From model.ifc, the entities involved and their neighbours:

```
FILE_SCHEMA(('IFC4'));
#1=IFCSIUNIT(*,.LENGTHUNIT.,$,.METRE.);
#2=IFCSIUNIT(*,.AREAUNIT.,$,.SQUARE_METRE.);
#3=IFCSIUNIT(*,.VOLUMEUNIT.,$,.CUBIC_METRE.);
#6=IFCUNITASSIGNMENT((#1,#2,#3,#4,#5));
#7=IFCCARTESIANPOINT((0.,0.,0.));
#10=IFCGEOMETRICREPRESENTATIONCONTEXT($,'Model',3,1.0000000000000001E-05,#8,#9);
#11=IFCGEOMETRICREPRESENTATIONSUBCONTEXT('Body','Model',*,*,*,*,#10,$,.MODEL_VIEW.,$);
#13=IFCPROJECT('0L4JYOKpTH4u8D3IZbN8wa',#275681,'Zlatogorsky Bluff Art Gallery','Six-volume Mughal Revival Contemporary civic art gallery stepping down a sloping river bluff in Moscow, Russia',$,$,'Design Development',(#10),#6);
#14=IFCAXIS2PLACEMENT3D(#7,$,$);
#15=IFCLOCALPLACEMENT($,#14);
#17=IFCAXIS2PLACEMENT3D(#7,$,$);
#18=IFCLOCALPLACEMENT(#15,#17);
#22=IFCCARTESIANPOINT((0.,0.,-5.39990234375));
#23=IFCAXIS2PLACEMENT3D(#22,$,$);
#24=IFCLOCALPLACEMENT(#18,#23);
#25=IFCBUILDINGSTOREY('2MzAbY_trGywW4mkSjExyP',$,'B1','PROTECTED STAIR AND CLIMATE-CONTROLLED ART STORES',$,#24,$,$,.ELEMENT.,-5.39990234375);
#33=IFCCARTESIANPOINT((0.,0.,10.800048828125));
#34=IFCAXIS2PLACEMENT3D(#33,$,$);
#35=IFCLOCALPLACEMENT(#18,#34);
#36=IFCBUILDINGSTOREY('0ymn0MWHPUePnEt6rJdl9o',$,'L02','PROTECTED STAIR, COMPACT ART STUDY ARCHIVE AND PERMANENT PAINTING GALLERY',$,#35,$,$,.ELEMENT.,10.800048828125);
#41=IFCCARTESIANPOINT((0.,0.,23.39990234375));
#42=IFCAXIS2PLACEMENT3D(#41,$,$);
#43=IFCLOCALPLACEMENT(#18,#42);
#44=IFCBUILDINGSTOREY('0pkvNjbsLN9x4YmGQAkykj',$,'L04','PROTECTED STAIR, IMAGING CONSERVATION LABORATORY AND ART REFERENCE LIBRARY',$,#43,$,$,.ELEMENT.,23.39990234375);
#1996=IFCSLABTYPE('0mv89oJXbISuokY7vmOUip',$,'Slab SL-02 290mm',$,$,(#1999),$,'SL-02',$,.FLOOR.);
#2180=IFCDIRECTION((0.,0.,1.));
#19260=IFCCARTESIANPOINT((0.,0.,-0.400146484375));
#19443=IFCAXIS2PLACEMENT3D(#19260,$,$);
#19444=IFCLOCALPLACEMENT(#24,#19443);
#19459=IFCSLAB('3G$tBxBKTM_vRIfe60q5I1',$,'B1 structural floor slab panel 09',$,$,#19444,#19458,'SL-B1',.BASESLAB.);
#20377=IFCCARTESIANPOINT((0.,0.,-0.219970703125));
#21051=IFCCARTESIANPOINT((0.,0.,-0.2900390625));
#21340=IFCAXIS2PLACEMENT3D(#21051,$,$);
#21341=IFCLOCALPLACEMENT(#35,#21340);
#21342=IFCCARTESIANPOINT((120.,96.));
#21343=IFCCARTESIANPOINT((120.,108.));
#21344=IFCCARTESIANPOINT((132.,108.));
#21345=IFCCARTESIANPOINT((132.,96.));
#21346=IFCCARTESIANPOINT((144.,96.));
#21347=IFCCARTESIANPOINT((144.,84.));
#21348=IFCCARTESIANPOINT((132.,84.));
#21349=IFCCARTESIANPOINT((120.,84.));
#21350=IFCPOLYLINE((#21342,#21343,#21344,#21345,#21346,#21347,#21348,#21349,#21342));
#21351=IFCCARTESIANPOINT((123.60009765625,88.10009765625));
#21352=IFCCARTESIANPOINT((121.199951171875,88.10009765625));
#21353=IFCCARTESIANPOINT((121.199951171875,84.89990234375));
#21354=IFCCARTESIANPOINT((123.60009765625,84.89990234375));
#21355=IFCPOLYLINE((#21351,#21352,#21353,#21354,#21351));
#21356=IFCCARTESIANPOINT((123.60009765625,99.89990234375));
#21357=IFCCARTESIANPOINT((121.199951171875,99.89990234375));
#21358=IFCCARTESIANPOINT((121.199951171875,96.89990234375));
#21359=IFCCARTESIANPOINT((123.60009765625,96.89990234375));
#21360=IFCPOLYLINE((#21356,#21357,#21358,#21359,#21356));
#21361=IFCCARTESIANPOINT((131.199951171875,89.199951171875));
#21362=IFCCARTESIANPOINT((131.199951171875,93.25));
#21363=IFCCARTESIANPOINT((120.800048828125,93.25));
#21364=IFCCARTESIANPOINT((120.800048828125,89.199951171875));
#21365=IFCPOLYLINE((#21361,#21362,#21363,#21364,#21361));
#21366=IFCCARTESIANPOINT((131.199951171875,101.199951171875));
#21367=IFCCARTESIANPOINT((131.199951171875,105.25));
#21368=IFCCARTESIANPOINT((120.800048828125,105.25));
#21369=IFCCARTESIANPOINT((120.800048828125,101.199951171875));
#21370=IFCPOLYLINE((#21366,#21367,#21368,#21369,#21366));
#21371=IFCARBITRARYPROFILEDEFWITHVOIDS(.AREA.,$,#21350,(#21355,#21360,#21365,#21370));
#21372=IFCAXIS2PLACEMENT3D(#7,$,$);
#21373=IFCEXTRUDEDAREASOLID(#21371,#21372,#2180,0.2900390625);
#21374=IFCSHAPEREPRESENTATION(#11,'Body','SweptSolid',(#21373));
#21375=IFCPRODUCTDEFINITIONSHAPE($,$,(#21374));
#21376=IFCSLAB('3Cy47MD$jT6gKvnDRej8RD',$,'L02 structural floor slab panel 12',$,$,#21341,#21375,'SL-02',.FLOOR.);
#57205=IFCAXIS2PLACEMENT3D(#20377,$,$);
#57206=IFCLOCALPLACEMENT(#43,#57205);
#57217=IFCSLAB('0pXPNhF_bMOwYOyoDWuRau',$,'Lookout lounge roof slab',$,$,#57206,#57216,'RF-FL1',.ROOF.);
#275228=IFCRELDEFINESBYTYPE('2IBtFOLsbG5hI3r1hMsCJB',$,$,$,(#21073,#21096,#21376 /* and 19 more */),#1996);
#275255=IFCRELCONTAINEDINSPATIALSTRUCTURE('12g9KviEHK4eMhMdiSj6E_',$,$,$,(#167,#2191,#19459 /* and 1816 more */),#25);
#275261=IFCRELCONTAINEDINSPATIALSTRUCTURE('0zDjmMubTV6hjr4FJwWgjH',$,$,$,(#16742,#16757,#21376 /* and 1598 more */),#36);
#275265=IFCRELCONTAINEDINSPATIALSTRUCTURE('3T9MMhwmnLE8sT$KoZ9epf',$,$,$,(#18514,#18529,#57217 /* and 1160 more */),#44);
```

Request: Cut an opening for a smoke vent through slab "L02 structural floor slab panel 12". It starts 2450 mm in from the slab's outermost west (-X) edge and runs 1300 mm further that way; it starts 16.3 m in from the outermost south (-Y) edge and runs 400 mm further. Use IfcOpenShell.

```python
import numpy as np
import ifcopenshell
import ifcopenshell.api.feature
import ifcopenshell.api.geometry
import ifcopenshell.api.root
import ifcopenshell.geom
import ifcopenshell.util.placement
import ifcopenshell.util.representation
import ifcopenshell.util.shape
import ifcopenshell.util.unit

model = ifcopenshell.open("model.ifc")
unit_scale = ifcopenshell.util.unit.calculate_unit_scale(model)
settings = ifcopenshell.geom.settings()


def volume(element):
    """Net volume in cubic metres, openings subtracted."""
    shape = ifcopenshell.geom.create_shape(settings, element)
    return ifcopenshell.util.shape.get_volume(shape.geometry)


slab = model.by_guid("3Cy47MD$jT6gKvnDRej8RD")
before = volume(slab)

# Extent in the slab's own axes, in metres. The edges named are its -X and -Y sides.
slab_shape = ifcopenshell.geom.create_shape(settings, slab)
vertices = ifcopenshell.util.shape.get_vertices(slab_shape.geometry)
x_min, y_min, bottom = vertices.min(axis=0)
top = vertices[:, 2].max()

opening = ifcopenshell.api.root.create_entity(model, ifc_class="IfcOpeningElement", name="Smoke vent opening", predefined_type="OPENING")
context = ifcopenshell.util.representation.get_context(model, "Model", "Body", "MODEL_VIEW")
width, depth = 1.3, 0.4
outline = [(0.0, 0.0), (width, 0.0), (width, depth), (0.0, depth), (0.0, 0.0)]
# Overshoot both faces by 50 mm so the cut is clean.
shape = ifcopenshell.api.geometry.add_slab_representation(
    model, context=context, depth=top - bottom + 0.1, polyline=outline
)
ifcopenshell.api.geometry.assign_representation(model, product=opening, representation=shape)

matrix = ifcopenshell.util.placement.get_local_placement(slab.ObjectPlacement)
matrix[:, 3] = matrix @ np.append(np.array([x_min + 2.45, y_min + 16.3, bottom - 0.05]) / unit_scale, 1.0)
ifcopenshell.api.geometry.edit_object_placement(model, product=opening, matrix=matrix, is_si=False)
ifcopenshell.api.feature.add_feature(model, feature=opening, element=slab)

after = volume(slab)

print(f"slab volume {before:.3f} -> {after:.3f} m3")

model.write("model_edited.ifc")
```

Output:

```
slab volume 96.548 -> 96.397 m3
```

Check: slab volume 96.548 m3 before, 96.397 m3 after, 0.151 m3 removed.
